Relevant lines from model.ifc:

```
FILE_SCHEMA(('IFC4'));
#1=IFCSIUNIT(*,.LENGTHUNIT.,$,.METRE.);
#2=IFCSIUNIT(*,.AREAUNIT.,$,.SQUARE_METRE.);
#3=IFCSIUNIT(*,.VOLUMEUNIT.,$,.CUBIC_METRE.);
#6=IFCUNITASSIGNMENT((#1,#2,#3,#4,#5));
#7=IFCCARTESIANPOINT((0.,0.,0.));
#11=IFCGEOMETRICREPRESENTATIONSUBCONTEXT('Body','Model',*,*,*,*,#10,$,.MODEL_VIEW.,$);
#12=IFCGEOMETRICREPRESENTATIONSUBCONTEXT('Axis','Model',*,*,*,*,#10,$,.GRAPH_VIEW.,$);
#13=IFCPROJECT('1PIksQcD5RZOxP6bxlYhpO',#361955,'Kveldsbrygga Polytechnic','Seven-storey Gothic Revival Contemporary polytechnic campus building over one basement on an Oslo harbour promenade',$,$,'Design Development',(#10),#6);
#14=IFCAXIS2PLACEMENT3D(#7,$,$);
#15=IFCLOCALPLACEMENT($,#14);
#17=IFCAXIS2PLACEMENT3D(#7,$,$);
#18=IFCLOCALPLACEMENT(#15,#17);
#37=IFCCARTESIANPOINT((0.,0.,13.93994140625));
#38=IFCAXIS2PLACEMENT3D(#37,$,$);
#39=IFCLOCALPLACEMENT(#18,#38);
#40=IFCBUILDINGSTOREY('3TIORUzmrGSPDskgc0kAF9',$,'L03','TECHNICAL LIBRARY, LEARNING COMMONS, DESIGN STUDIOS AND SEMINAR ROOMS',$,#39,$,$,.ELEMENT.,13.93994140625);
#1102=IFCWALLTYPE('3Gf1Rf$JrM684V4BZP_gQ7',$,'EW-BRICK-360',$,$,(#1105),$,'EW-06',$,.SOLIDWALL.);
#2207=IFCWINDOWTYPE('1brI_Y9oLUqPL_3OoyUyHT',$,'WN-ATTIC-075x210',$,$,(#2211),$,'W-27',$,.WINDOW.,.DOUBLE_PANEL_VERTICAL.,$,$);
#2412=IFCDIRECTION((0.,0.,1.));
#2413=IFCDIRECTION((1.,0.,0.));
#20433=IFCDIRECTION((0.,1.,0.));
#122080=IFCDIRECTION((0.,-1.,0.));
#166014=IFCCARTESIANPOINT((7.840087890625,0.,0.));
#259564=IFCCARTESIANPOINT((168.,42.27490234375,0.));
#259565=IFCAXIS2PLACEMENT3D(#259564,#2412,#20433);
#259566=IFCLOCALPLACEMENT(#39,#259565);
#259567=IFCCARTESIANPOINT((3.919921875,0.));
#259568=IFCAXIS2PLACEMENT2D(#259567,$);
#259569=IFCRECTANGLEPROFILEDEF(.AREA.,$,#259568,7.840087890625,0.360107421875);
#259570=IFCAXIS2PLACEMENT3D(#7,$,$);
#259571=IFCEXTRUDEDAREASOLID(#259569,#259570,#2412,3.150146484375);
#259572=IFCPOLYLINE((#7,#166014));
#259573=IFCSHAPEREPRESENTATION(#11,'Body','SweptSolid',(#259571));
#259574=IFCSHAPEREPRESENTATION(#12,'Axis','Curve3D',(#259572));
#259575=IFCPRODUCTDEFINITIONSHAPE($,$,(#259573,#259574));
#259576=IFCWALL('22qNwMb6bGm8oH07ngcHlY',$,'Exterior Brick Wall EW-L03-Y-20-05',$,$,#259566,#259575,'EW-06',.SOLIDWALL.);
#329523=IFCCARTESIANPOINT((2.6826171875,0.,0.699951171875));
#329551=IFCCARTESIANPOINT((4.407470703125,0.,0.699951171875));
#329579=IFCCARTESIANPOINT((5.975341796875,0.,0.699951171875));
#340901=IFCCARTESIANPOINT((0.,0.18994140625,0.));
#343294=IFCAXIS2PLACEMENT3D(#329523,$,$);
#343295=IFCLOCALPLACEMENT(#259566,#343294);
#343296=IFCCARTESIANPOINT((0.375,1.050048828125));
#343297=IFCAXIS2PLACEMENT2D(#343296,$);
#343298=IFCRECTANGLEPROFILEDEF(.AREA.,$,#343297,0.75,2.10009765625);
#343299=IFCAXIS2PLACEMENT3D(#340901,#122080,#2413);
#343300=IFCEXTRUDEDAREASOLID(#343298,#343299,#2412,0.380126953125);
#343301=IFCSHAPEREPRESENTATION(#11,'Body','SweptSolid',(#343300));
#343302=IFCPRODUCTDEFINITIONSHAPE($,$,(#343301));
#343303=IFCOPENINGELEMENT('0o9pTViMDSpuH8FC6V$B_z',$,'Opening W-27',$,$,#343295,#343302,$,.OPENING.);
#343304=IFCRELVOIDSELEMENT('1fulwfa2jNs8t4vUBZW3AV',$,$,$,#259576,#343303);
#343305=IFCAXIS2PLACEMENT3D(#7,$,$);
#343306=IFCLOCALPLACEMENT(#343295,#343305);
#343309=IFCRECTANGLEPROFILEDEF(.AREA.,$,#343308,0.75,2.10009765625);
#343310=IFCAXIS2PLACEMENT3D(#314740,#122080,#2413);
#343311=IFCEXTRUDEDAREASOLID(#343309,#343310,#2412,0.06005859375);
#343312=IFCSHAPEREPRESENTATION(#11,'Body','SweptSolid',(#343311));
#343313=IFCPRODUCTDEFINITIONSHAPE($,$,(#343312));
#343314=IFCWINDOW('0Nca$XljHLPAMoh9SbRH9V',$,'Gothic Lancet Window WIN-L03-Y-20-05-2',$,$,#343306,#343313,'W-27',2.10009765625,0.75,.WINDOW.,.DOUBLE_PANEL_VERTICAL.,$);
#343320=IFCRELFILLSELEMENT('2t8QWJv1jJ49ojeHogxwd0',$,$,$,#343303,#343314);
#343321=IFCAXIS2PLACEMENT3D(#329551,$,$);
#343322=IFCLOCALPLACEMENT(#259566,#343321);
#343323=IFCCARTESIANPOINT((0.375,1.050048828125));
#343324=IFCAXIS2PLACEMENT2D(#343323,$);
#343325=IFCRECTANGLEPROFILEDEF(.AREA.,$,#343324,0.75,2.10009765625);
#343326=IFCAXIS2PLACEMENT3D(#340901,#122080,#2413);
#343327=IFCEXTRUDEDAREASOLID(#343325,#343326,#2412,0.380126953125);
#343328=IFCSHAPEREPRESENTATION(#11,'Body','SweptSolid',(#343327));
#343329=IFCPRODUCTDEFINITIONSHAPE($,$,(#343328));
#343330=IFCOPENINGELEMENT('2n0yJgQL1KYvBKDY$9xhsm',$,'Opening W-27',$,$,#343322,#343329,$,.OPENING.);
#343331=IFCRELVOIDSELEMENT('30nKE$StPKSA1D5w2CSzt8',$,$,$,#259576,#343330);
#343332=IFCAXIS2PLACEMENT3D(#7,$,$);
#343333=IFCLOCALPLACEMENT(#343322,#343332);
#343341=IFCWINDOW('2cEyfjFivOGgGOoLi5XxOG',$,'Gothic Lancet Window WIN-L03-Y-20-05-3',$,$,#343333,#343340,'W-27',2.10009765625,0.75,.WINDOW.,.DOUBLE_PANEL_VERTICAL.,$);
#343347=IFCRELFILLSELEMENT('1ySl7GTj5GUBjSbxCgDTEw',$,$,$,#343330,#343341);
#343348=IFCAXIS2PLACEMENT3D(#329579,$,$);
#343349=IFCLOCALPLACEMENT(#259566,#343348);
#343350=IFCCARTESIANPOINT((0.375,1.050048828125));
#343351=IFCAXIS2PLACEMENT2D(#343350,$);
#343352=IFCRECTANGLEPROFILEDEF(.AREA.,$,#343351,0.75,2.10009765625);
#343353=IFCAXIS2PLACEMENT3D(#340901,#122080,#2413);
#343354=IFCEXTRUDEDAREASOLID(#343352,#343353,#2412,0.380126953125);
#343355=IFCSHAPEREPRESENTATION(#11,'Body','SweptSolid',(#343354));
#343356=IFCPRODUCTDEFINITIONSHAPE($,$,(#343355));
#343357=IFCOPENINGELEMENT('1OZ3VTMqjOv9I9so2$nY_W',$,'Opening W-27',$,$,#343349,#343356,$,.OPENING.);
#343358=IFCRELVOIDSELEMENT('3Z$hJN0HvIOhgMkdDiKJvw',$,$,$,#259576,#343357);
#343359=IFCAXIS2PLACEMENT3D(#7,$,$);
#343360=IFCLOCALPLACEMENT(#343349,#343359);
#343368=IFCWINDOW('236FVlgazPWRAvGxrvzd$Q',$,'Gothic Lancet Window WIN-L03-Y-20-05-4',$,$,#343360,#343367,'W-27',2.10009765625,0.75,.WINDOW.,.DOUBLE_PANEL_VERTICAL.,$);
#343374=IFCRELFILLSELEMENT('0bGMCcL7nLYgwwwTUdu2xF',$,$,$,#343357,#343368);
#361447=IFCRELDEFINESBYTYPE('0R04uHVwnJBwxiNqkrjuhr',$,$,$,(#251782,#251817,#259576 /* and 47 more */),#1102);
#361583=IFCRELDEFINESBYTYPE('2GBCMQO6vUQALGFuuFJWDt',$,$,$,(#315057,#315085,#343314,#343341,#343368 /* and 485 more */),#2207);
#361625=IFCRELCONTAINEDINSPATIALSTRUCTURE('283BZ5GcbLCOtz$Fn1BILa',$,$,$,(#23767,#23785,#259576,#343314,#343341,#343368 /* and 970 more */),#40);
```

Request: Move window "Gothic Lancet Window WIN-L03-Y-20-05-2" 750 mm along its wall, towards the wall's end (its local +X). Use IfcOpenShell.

```python
import ifcopenshell
import ifcopenshell.api.geometry
import ifcopenshell.util.placement
import ifcopenshell.util.unit

model = ifcopenshell.open("model.ifc")
unit_scale = ifcopenshell.util.unit.calculate_unit_scale(model)

window = model.by_guid("0Nca$XljHLPAMoh9SbRH9V")
opening = window.FillsVoids[0].RelatingOpeningElement
wall = opening.VoidsElements[0].RelatingBuildingElement

wall_matrix = ifcopenshell.util.placement.get_local_placement(wall.ObjectPlacement)
shift = wall_matrix[:3, 0] * 0.75 / unit_scale
before = ifcopenshell.util.placement.get_local_placement(window.ObjectPlacement)[:3, 3].copy()

# The window is placed relative to its opening, so it follows when the opening moves.
matrix = ifcopenshell.util.placement.get_local_placement(opening.ObjectPlacement)
matrix[:3, 3] += shift
ifcopenshell.api.geometry.edit_object_placement(
    model, product=opening, matrix=matrix, is_si=False, should_transform_children=True
)

after = ifcopenshell.util.placement.get_local_placement(window.ObjectPlacement)[:3, 3]
print("window moved by", (after - before).round(3) + 0.0)

model.write("model_edited.ifc")
```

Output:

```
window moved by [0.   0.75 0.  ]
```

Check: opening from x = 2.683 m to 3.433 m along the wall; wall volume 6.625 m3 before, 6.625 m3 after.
